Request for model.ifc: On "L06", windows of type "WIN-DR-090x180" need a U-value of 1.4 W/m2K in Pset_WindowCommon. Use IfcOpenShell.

First a look at what the model holds.

```python
import ifcopenshell
import ifcopenshell.util.element

model = ifcopenshell.open("model.ifc")
print(model.schema)
storey = next(s for s in model.by_type("IfcBuildingStorey") if s.Name == "L06")
windows = [e for e in ifcopenshell.util.element.get_decomposition(storey) if e.is_a("IfcWindow")]
seen = {}
for e in windows:
    element_type = ifcopenshell.util.element.get_type(e)
    key = (element_type.Name if element_type != e and element_type else None, ifcopenshell.util.element.get_pset(e, "Pset_WindowCommon", "ThermalTransmittance"))
    seen[key] = seen.get(key, 0) + 1
for (name, value), count in sorted(seen.items(), key=str):
    print(count, "x", name, "|", value)
```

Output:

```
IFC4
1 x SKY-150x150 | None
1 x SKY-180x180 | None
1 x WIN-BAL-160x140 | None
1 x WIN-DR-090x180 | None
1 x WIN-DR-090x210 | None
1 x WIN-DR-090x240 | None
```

```python
import ifcopenshell
import ifcopenshell.api.pset
import ifcopenshell.util.element

model = ifcopenshell.open("model.ifc")

storey = next(s for s in model.by_type("IfcBuildingStorey") if s.Name == "L06")
windows = [e for e in ifcopenshell.util.element.get_decomposition(storey) if e.is_a("IfcWindow")]

count = 0
for e in windows:
    element_type = ifcopenshell.util.element.get_type(e)
    if element_type in (None, e) or element_type.Name != "WIN-DR-090x180":
        continue
    # add_pset returns the element's existing set when there is one.
    pset = ifcopenshell.api.pset.add_pset(model, product=e, name="Pset_WindowCommon")
    ifcopenshell.api.pset.edit_pset(model, pset=pset, properties={"ThermalTransmittance": 1.4})
    count += 1

print(count, "windows updated")

model.write("model_rev.ifc")
```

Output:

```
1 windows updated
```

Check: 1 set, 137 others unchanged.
